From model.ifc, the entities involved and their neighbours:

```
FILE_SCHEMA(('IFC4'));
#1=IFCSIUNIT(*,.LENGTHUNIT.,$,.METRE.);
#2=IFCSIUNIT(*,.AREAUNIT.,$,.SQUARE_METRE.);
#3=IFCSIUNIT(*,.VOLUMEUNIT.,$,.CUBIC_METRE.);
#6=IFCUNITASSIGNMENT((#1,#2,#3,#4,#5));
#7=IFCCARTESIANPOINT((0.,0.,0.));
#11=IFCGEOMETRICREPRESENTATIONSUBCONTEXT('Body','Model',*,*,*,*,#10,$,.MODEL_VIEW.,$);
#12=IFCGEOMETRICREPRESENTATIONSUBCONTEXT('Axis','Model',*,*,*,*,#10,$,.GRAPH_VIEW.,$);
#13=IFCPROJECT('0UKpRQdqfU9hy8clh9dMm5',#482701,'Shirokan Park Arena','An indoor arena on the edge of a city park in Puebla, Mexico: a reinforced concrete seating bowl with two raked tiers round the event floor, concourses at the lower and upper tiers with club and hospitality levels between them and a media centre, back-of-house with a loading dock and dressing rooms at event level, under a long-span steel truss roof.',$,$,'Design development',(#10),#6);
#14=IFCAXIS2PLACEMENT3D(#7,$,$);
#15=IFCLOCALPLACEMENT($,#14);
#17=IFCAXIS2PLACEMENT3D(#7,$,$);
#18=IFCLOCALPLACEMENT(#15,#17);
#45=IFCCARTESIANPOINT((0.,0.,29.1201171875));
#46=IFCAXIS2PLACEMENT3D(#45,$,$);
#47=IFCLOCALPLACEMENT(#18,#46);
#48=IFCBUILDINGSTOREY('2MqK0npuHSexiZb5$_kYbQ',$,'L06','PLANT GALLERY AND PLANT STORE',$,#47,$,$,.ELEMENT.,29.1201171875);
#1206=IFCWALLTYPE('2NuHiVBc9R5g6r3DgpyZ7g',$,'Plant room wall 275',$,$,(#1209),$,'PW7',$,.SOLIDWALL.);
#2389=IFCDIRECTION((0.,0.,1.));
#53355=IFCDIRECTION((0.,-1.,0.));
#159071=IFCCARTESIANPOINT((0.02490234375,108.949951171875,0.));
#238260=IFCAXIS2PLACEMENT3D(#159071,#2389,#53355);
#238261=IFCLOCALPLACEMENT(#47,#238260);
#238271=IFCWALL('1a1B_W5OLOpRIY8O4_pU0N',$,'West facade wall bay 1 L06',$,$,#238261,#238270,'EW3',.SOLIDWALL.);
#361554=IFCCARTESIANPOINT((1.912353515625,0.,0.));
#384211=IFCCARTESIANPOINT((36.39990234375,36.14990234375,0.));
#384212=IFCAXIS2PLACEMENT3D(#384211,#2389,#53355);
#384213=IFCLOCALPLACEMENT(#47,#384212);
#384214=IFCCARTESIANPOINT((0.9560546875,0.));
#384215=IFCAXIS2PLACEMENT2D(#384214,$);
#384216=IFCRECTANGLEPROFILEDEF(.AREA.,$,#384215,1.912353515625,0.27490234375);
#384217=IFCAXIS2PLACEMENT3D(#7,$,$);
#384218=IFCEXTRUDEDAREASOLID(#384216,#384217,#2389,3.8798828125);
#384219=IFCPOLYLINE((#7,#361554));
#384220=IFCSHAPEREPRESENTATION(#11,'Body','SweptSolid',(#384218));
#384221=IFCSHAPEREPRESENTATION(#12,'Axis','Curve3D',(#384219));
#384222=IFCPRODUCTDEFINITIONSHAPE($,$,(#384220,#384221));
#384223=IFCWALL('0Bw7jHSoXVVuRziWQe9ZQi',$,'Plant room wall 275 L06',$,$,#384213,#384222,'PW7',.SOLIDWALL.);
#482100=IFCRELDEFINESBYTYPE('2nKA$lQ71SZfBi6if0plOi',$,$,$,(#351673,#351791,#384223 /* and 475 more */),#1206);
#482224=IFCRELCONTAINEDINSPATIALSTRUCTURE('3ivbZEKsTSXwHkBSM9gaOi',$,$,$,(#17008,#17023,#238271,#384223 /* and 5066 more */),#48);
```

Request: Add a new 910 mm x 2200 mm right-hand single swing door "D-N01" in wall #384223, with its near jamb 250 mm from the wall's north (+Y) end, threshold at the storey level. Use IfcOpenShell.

```python
import numpy as np
import ifcopenshell
import ifcopenshell.api.feature
import ifcopenshell.api.geometry
import ifcopenshell.api.root
import ifcopenshell.api.spatial
import ifcopenshell.geom
import ifcopenshell.util.element
import ifcopenshell.util.placement
import ifcopenshell.util.representation
import ifcopenshell.util.shape
import ifcopenshell.util.unit

model = ifcopenshell.open("model.ifc")
unit_scale = ifcopenshell.util.unit.calculate_unit_scale(model)
settings = ifcopenshell.geom.settings()


def volume(element):
    """Net volume in cubic metres, openings subtracted."""
    shape = ifcopenshell.geom.create_shape(settings, element)
    return ifcopenshell.util.shape.get_volume(shape.geometry)


wall = model.by_guid("0Bw7jHSoXVVuRziWQe9ZQi")
storey = ifcopenshell.util.element.get_container(wall, ifc_class="IfcBuildingStorey")
context = ifcopenshell.util.representation.get_context(model, "Model", "Body", "MODEL_VIEW")
before = volume(wall)

width, height, from_end, sill = 0.91, 2.2, 0.25, 0.0  # metres

# The wall runs along its own X axis, and the end named is its -X end.
wall_shape = ifcopenshell.geom.create_shape(settings, wall)
x, y, z = ifcopenshell.util.shape.get_vertices(wall_shape.geometry).T
start = x.min() + from_end
face, thickness = float(y.min()), float(y.max() - y.min())
wall_matrix = ifcopenshell.util.placement.get_local_placement(wall.ObjectPlacement)
level = ifcopenshell.util.placement.get_local_placement(storey.ObjectPlacement)[2, 3]


def in_wall(x, y):
    """Placement at x, y metres in the wall's axes, at sill height."""
    matrix = wall_matrix.copy()
    matrix[:, 3] = wall_matrix @ np.array([x / unit_scale, y / unit_scale, 0.0, 1.0])
    matrix[2, 3] = level + sill / unit_scale
    return matrix


# Opening: a box that overshoots both wall faces by 50 mm.
opening = ifcopenshell.api.root.create_entity(model, ifc_class="IfcOpeningElement", predefined_type="OPENING")
box = ifcopenshell.api.geometry.add_wall_representation(
    model, context=context, length=width, height=height, thickness=thickness + 0.1
)
ifcopenshell.api.geometry.assign_representation(model, product=opening, representation=box)
ifcopenshell.api.geometry.edit_object_placement(model, product=opening, matrix=in_wall(start, face - 0.05), is_si=False)
ifcopenshell.api.feature.add_feature(model, feature=opening, element=wall)

door = ifcopenshell.api.root.create_entity(model, ifc_class="IfcDoor", name="D-N01", predefined_type="DOOR")
door.OverallWidth, door.OverallHeight = width / unit_scale, height / unit_scale
door.OperationType = "SINGLE_SWING_RIGHT"
body = ifcopenshell.api.geometry.add_door_representation(
    model,
    context=context,
    overall_width=door.OverallWidth,
    overall_height=door.OverallHeight,
    operation_type="SINGLE_SWING_RIGHT",
    lining_properties={"LiningDepth": thickness / unit_scale, "ThresholdDepth": thickness / unit_scale},
)
ifcopenshell.api.geometry.assign_representation(model, product=door, representation=body)
ifcopenshell.api.spatial.assign_container(model, products=[door], relating_structure=storey)
ifcopenshell.api.feature.add_filling(model, opening=opening, element=door)

# The lining spans the wall, so the door starts at the wall face.
ifcopenshell.api.geometry.edit_object_placement(model, product=door, matrix=in_wall(start, face), is_si=False)

after = volume(wall)

print(f"wall volume {before:.3f} -> {after:.3f} m3")

model.write("model_rev.ifc")
```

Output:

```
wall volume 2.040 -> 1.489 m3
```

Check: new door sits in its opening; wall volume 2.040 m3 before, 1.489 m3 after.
